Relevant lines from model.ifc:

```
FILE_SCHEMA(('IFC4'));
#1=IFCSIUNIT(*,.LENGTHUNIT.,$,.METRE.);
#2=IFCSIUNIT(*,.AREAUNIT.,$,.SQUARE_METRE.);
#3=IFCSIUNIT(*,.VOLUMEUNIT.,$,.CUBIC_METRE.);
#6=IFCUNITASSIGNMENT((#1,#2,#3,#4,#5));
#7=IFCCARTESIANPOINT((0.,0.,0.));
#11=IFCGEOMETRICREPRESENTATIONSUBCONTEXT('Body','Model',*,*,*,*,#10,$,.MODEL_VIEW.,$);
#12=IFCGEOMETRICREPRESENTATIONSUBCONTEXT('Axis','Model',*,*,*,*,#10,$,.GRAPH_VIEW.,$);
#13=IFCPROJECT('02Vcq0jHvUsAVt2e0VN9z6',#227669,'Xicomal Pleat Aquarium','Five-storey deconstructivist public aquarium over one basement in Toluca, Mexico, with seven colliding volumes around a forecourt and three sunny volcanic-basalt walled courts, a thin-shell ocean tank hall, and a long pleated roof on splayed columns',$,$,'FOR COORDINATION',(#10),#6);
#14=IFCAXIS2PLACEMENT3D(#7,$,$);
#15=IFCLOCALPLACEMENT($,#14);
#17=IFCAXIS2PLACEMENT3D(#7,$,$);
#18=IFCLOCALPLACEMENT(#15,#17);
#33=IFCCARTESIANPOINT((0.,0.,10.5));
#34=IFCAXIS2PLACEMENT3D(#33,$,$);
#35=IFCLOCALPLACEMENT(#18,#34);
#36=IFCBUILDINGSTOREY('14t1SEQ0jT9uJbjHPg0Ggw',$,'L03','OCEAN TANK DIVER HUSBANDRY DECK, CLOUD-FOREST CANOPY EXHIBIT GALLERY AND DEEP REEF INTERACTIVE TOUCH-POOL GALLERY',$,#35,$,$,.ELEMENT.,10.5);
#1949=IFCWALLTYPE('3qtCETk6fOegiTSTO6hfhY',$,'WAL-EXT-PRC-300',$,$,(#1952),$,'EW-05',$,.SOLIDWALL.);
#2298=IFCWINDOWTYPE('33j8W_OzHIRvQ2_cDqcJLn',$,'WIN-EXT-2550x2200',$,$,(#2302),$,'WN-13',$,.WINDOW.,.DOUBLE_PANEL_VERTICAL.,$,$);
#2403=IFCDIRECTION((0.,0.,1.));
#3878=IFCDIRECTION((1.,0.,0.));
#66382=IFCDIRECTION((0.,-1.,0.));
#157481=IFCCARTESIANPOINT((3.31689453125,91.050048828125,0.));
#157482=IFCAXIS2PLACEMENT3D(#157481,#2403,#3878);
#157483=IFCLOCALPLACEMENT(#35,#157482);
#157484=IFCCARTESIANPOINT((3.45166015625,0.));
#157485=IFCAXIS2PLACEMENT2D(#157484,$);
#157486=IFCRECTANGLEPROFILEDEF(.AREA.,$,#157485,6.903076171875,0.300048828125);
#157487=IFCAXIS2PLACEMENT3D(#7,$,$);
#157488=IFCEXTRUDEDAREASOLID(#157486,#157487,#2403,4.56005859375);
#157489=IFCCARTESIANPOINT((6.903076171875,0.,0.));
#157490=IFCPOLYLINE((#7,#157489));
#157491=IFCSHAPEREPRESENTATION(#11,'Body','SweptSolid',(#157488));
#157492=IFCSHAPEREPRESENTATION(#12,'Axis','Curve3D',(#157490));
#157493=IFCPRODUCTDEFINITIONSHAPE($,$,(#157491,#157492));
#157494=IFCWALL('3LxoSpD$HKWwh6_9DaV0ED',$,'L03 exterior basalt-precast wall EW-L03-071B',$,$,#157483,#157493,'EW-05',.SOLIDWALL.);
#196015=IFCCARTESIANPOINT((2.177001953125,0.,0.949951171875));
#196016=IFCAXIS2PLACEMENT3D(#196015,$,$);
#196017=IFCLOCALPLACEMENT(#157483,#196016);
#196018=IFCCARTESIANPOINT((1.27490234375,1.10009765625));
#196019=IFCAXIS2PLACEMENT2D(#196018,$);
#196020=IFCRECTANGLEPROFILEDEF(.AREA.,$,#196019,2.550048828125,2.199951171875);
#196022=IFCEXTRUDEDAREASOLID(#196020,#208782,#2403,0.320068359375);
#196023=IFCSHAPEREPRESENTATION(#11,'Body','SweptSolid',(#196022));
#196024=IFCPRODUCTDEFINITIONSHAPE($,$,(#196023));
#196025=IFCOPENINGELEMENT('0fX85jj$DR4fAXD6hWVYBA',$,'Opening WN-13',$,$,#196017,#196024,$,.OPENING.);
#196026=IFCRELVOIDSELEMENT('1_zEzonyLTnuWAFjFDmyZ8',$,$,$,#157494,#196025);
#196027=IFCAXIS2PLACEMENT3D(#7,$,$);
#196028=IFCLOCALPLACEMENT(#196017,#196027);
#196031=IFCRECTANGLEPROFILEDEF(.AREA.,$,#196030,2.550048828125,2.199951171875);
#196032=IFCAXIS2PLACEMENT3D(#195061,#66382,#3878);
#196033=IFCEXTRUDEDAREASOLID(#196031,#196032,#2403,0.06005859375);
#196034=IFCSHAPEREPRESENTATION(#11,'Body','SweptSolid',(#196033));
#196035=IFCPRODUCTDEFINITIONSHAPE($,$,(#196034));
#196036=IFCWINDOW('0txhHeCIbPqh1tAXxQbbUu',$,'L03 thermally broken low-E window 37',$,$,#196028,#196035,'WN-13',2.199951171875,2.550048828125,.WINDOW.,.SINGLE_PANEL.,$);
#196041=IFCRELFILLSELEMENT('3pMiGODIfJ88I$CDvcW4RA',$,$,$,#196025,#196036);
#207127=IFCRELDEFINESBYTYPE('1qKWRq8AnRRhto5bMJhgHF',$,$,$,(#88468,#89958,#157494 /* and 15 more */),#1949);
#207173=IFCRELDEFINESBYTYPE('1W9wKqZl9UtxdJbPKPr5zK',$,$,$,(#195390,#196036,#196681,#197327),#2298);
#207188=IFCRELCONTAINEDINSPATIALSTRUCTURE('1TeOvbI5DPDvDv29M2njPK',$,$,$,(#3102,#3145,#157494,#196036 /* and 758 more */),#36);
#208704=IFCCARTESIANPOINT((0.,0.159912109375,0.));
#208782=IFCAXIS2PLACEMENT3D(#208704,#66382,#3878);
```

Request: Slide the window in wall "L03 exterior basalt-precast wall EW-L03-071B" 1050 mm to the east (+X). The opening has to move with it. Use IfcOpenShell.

```python
import ifcopenshell
import ifcopenshell.api.geometry
import ifcopenshell.util.placement

model = ifcopenshell.open("model.ifc")

window = model.by_guid("0txhHeCIbPqh1tAXxQbbUu")
opening = window.FillsVoids[0].RelatingOpeningElement
wall = opening.VoidsElements[0].RelatingBuildingElement

wall_matrix = ifcopenshell.util.placement.get_local_placement(wall.ObjectPlacement)
shift = wall_matrix[:3, 0] * 1.05
before = ifcopenshell.util.placement.get_local_placement(window.ObjectPlacement)[:3, 3].copy()

# The window is placed relative to its opening, so it follows when the opening moves.
matrix = ifcopenshell.util.placement.get_local_placement(opening.ObjectPlacement)
matrix[:3, 3] += shift
ifcopenshell.api.geometry.edit_object_placement(
    model, product=opening, matrix=matrix, is_si=False, should_transform_children=True
)

after = ifcopenshell.util.placement.get_local_placement(window.ObjectPlacement)[:3, 3]
print("window moved by", (after - before).round(3) + 0.0)

model.write("model_v2.ifc")
```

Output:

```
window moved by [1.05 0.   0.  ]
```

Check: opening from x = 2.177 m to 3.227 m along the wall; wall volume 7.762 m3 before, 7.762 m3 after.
